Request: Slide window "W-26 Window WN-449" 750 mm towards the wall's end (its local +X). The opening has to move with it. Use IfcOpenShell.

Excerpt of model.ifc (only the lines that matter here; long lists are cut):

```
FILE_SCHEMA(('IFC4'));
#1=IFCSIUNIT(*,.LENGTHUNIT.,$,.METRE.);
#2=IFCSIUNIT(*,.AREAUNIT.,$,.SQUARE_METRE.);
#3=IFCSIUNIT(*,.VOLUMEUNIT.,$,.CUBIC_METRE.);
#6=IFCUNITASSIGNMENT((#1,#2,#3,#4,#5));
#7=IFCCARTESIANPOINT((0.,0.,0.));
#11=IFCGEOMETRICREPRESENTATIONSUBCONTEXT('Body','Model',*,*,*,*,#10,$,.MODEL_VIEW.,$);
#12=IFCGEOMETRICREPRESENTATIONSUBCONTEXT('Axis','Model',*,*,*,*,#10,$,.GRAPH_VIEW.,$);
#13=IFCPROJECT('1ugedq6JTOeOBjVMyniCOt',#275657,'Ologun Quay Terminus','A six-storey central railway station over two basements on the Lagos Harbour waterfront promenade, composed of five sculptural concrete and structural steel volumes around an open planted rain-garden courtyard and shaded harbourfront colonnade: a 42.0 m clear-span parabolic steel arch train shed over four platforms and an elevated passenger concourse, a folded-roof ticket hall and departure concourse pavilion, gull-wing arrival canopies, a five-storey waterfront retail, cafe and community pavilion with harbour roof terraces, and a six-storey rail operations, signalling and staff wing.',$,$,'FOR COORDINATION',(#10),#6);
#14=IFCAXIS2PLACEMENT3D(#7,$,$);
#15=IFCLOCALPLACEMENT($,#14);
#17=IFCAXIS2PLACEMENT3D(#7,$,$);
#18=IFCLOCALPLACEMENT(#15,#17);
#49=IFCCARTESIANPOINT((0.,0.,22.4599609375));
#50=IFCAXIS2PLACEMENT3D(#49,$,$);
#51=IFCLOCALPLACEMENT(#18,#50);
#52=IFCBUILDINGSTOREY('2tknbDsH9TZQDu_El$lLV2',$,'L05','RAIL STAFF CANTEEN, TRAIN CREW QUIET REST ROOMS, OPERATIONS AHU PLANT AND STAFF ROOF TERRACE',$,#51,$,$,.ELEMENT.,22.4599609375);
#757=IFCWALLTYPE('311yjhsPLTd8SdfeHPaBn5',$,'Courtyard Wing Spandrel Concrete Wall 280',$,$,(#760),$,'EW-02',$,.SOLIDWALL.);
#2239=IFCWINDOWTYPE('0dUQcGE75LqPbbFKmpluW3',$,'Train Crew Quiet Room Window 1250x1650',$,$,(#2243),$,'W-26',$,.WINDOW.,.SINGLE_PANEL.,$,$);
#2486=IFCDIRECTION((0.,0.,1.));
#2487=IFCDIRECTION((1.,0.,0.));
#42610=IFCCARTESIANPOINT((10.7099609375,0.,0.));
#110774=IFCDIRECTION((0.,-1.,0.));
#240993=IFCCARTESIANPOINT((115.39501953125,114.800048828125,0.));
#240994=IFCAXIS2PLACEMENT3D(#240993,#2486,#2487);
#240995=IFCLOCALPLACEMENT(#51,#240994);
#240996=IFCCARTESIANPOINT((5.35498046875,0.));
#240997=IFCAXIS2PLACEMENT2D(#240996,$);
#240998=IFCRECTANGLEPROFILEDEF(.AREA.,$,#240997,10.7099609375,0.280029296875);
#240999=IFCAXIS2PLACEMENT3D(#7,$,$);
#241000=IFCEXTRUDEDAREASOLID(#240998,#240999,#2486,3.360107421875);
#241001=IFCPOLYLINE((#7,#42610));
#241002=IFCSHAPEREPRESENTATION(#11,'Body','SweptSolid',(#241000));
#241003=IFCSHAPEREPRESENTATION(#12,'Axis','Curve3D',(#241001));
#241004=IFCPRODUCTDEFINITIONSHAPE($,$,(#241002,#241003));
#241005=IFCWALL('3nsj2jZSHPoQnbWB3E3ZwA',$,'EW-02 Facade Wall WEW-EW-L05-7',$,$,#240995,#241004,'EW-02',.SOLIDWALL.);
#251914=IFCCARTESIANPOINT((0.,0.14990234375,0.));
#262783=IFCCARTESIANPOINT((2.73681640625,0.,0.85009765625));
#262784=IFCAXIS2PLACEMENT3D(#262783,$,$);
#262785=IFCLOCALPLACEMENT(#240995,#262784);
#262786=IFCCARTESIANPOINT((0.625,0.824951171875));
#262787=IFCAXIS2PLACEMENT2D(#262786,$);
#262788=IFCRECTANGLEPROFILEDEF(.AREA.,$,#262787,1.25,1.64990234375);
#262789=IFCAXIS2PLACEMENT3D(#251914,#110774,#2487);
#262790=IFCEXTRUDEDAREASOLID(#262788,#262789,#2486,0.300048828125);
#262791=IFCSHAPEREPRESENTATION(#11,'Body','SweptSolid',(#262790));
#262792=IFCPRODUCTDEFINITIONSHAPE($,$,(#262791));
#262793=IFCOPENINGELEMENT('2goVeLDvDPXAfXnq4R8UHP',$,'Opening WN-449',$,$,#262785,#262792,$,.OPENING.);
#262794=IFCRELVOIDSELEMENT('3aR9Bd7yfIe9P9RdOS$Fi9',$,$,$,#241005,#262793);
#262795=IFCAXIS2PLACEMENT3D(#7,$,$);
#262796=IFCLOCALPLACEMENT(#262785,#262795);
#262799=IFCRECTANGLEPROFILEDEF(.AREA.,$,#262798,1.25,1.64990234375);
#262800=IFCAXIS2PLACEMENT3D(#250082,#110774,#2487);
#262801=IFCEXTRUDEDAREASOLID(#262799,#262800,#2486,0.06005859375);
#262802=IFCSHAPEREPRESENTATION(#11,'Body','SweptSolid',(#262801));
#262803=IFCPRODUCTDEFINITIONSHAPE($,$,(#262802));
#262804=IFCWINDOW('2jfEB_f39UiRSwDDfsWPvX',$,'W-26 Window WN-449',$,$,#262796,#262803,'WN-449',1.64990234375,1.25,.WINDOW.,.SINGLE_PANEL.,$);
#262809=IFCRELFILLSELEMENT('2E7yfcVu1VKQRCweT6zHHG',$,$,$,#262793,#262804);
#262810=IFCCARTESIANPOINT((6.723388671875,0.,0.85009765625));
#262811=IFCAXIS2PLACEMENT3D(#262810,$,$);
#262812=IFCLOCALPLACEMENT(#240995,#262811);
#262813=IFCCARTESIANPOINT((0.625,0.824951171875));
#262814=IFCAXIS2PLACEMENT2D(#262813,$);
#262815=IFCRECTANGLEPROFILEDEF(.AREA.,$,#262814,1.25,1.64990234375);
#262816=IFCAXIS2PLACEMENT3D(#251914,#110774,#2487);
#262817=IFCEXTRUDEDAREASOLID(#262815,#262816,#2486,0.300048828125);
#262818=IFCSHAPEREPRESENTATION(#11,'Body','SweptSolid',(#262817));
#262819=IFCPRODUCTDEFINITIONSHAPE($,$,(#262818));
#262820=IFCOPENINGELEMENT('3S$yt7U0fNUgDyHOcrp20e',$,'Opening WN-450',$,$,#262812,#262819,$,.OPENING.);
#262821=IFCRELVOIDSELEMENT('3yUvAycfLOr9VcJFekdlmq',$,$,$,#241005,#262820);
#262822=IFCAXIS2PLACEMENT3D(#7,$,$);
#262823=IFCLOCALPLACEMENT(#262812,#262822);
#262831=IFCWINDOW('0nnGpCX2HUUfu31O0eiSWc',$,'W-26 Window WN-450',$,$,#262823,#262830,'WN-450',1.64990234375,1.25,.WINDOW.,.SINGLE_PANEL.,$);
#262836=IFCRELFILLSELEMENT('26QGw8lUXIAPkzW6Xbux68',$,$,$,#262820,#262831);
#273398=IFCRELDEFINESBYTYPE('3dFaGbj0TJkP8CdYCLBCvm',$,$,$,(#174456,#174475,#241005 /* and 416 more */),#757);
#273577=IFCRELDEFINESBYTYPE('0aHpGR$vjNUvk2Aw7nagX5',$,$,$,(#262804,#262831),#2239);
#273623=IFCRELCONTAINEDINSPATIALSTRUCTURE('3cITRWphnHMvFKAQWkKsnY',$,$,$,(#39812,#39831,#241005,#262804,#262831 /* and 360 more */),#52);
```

```python
import ifcopenshell
import ifcopenshell.api.geometry
import ifcopenshell.util.placement

model = ifcopenshell.open("model.ifc")

window = model.by_guid("2jfEB_f39UiRSwDDfsWPvX")
opening = window.FillsVoids[0].RelatingOpeningElement
wall = opening.VoidsElements[0].RelatingBuildingElement

wall_matrix = ifcopenshell.util.placement.get_local_placement(wall.ObjectPlacement)
shift = wall_matrix[:3, 0] * 0.75
before = ifcopenshell.util.placement.get_local_placement(window.ObjectPlacement)[:3, 3].copy()

# The window is placed relative to its opening, so it follows when the opening moves.
matrix = ifcopenshell.util.placement.get_local_placement(opening.ObjectPlacement)
matrix[:3, 3] += shift
ifcopenshell.api.geometry.edit_object_placement(
    model, product=opening, matrix=matrix, is_si=False, should_transform_children=True
)

after = ifcopenshell.util.placement.get_local_placement(window.ObjectPlacement)[:3, 3]
print("window moved by", (after - before).round(3) + 0.0)

model.write("model_v2.ifc")
```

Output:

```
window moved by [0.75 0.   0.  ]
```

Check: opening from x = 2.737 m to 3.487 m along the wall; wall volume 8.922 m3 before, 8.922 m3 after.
